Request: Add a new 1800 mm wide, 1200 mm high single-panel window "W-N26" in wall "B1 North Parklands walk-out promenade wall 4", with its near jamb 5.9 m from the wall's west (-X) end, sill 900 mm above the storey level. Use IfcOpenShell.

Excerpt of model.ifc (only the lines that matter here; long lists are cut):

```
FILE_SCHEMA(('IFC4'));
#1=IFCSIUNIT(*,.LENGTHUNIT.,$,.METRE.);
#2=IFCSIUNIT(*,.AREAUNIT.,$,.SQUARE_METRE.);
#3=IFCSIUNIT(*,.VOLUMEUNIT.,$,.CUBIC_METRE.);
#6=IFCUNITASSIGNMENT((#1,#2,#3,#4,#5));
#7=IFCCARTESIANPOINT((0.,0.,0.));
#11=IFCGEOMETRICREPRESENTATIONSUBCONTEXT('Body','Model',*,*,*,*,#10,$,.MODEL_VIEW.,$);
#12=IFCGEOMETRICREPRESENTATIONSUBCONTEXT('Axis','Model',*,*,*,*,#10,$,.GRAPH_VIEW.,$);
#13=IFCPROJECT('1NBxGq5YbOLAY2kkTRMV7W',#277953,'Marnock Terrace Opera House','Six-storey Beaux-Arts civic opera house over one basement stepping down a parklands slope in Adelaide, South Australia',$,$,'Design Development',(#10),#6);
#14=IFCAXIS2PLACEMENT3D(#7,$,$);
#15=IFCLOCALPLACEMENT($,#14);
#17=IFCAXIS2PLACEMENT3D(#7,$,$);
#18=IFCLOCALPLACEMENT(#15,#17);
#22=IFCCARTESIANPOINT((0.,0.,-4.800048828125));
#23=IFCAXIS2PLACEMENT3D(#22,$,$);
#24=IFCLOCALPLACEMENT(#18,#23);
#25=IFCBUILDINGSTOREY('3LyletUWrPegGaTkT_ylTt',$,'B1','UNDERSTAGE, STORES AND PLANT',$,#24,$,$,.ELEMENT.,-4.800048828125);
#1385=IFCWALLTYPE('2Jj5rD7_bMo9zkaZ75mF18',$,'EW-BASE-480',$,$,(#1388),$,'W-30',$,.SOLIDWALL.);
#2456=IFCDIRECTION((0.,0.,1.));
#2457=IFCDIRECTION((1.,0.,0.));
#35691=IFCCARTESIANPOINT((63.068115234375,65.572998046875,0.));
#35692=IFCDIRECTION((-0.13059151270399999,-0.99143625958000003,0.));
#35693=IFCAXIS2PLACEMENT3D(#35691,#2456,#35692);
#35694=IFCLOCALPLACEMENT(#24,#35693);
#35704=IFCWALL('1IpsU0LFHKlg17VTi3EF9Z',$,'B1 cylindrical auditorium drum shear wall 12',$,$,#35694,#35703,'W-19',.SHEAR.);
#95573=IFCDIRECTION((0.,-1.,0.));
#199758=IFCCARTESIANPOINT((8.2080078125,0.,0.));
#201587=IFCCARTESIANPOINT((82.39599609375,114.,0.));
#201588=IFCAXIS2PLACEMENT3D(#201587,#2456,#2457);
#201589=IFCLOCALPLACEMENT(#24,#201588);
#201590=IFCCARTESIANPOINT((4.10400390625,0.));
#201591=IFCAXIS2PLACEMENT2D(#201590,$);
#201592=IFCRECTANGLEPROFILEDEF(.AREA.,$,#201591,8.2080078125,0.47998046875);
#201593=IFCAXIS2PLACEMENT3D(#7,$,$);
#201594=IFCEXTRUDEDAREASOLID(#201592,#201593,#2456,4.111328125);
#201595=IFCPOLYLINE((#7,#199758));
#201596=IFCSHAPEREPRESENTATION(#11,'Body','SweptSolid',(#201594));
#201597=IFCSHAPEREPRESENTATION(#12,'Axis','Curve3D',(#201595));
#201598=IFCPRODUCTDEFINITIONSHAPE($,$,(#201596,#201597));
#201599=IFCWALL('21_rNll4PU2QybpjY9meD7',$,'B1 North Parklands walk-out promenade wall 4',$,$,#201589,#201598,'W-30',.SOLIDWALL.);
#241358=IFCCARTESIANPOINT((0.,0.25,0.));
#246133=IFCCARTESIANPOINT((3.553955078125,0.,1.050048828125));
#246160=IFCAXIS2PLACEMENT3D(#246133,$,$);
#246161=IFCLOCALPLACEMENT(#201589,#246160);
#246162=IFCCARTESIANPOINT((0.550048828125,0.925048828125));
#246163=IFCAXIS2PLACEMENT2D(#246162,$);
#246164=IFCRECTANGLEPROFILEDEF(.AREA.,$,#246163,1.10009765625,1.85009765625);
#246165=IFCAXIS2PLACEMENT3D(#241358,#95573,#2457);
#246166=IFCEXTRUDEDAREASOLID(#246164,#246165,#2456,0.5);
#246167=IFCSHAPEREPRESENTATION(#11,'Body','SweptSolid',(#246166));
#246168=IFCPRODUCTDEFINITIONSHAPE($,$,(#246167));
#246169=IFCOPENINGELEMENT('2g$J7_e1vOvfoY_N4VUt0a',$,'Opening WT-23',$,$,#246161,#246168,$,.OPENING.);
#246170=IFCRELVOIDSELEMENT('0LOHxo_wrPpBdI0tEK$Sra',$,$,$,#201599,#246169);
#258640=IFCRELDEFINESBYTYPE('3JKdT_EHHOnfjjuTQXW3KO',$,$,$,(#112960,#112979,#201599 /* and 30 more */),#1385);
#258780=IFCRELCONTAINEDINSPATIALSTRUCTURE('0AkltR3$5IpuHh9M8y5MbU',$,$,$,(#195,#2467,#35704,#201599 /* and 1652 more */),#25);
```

```python
import numpy as np
import ifcopenshell
import ifcopenshell.api.feature
import ifcopenshell.api.geometry
import ifcopenshell.api.root
import ifcopenshell.api.spatial
import ifcopenshell.geom
import ifcopenshell.util.element
import ifcopenshell.util.placement
import ifcopenshell.util.representation
import ifcopenshell.util.shape
import ifcopenshell.util.unit

model = ifcopenshell.open("model.ifc")
unit_scale = ifcopenshell.util.unit.calculate_unit_scale(model)
settings = ifcopenshell.geom.settings()


def volume(element):
    """Net volume in cubic metres, openings subtracted."""
    shape = ifcopenshell.geom.create_shape(settings, element)
    return ifcopenshell.util.shape.get_volume(shape.geometry)


wall = model.by_guid("21_rNll4PU2QybpjY9meD7")
storey = ifcopenshell.util.element.get_container(wall, ifc_class="IfcBuildingStorey")
context = ifcopenshell.util.representation.get_context(model, "Model", "Body", "MODEL_VIEW")
before = volume(wall)

width, height, from_end, sill = 1.8, 1.2, 5.9, 0.9  # metres

# The wall runs along its own X axis, and the end named is its -X end.
wall_shape = ifcopenshell.geom.create_shape(settings, wall)
x, y, z = ifcopenshell.util.shape.get_vertices(wall_shape.geometry).T
start = x.min() + from_end
face, thickness = float(y.min()), float(y.max() - y.min())
wall_matrix = ifcopenshell.util.placement.get_local_placement(wall.ObjectPlacement)
level = ifcopenshell.util.placement.get_local_placement(storey.ObjectPlacement)[2, 3]


def in_wall(x, y):
    """Placement at x, y metres in the wall's axes, at sill height."""
    matrix = wall_matrix.copy()
    matrix[:, 3] = wall_matrix @ np.array([x / unit_scale, y / unit_scale, 0.0, 1.0])
    matrix[2, 3] = level + sill / unit_scale
    return matrix


# Opening: a box that overshoots both wall faces by 50 mm.
opening = ifcopenshell.api.root.create_entity(model, ifc_class="IfcOpeningElement", predefined_type="OPENING")
box = ifcopenshell.api.geometry.add_wall_representation(
    model, context=context, length=width, height=height, thickness=thickness + 0.1
)
ifcopenshell.api.geometry.assign_representation(model, product=opening, representation=box)
ifcopenshell.api.geometry.edit_object_placement(model, product=opening, matrix=in_wall(start, face - 0.05), is_si=False)
ifcopenshell.api.feature.add_feature(model, feature=opening, element=wall)

window = ifcopenshell.api.root.create_entity(model, ifc_class="IfcWindow", name="W-N26", predefined_type="WINDOW")
window.OverallWidth, window.OverallHeight = width / unit_scale, height / unit_scale
window.PartitioningType = "SINGLE_PANEL"
body = ifcopenshell.api.geometry.add_window_representation(
    model,
    context=context,
    overall_width=window.OverallWidth,
    overall_height=window.OverallHeight,
    partition_type="SINGLE_PANEL",
)
ifcopenshell.api.geometry.assign_representation(model, product=window, representation=body)
ifcopenshell.api.spatial.assign_container(model, products=[window], relating_structure=storey)
ifcopenshell.api.feature.add_filling(model, opening=opening, element=window)

# Centre the window in the wall's thickness.
ifcopenshell.api.geometry.edit_object_placement(model, product=window, matrix=in_wall(start, face), is_si=False)
window_shape = ifcopenshell.geom.create_shape(settings, window)
depth = ifcopenshell.util.shape.get_vertices(window_shape.geometry)[:, 1]
offset = face + thickness / 2 - (depth.min() + depth.max()) / 2
ifcopenshell.api.geometry.edit_object_placement(model, product=window, matrix=in_wall(start, offset), is_si=False)

after = volume(wall)

print(f"wall volume {before:.3f} -> {after:.3f} m3")

model.write("model_updated.ifc")
```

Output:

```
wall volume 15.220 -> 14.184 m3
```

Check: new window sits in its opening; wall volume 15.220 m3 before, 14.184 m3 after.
